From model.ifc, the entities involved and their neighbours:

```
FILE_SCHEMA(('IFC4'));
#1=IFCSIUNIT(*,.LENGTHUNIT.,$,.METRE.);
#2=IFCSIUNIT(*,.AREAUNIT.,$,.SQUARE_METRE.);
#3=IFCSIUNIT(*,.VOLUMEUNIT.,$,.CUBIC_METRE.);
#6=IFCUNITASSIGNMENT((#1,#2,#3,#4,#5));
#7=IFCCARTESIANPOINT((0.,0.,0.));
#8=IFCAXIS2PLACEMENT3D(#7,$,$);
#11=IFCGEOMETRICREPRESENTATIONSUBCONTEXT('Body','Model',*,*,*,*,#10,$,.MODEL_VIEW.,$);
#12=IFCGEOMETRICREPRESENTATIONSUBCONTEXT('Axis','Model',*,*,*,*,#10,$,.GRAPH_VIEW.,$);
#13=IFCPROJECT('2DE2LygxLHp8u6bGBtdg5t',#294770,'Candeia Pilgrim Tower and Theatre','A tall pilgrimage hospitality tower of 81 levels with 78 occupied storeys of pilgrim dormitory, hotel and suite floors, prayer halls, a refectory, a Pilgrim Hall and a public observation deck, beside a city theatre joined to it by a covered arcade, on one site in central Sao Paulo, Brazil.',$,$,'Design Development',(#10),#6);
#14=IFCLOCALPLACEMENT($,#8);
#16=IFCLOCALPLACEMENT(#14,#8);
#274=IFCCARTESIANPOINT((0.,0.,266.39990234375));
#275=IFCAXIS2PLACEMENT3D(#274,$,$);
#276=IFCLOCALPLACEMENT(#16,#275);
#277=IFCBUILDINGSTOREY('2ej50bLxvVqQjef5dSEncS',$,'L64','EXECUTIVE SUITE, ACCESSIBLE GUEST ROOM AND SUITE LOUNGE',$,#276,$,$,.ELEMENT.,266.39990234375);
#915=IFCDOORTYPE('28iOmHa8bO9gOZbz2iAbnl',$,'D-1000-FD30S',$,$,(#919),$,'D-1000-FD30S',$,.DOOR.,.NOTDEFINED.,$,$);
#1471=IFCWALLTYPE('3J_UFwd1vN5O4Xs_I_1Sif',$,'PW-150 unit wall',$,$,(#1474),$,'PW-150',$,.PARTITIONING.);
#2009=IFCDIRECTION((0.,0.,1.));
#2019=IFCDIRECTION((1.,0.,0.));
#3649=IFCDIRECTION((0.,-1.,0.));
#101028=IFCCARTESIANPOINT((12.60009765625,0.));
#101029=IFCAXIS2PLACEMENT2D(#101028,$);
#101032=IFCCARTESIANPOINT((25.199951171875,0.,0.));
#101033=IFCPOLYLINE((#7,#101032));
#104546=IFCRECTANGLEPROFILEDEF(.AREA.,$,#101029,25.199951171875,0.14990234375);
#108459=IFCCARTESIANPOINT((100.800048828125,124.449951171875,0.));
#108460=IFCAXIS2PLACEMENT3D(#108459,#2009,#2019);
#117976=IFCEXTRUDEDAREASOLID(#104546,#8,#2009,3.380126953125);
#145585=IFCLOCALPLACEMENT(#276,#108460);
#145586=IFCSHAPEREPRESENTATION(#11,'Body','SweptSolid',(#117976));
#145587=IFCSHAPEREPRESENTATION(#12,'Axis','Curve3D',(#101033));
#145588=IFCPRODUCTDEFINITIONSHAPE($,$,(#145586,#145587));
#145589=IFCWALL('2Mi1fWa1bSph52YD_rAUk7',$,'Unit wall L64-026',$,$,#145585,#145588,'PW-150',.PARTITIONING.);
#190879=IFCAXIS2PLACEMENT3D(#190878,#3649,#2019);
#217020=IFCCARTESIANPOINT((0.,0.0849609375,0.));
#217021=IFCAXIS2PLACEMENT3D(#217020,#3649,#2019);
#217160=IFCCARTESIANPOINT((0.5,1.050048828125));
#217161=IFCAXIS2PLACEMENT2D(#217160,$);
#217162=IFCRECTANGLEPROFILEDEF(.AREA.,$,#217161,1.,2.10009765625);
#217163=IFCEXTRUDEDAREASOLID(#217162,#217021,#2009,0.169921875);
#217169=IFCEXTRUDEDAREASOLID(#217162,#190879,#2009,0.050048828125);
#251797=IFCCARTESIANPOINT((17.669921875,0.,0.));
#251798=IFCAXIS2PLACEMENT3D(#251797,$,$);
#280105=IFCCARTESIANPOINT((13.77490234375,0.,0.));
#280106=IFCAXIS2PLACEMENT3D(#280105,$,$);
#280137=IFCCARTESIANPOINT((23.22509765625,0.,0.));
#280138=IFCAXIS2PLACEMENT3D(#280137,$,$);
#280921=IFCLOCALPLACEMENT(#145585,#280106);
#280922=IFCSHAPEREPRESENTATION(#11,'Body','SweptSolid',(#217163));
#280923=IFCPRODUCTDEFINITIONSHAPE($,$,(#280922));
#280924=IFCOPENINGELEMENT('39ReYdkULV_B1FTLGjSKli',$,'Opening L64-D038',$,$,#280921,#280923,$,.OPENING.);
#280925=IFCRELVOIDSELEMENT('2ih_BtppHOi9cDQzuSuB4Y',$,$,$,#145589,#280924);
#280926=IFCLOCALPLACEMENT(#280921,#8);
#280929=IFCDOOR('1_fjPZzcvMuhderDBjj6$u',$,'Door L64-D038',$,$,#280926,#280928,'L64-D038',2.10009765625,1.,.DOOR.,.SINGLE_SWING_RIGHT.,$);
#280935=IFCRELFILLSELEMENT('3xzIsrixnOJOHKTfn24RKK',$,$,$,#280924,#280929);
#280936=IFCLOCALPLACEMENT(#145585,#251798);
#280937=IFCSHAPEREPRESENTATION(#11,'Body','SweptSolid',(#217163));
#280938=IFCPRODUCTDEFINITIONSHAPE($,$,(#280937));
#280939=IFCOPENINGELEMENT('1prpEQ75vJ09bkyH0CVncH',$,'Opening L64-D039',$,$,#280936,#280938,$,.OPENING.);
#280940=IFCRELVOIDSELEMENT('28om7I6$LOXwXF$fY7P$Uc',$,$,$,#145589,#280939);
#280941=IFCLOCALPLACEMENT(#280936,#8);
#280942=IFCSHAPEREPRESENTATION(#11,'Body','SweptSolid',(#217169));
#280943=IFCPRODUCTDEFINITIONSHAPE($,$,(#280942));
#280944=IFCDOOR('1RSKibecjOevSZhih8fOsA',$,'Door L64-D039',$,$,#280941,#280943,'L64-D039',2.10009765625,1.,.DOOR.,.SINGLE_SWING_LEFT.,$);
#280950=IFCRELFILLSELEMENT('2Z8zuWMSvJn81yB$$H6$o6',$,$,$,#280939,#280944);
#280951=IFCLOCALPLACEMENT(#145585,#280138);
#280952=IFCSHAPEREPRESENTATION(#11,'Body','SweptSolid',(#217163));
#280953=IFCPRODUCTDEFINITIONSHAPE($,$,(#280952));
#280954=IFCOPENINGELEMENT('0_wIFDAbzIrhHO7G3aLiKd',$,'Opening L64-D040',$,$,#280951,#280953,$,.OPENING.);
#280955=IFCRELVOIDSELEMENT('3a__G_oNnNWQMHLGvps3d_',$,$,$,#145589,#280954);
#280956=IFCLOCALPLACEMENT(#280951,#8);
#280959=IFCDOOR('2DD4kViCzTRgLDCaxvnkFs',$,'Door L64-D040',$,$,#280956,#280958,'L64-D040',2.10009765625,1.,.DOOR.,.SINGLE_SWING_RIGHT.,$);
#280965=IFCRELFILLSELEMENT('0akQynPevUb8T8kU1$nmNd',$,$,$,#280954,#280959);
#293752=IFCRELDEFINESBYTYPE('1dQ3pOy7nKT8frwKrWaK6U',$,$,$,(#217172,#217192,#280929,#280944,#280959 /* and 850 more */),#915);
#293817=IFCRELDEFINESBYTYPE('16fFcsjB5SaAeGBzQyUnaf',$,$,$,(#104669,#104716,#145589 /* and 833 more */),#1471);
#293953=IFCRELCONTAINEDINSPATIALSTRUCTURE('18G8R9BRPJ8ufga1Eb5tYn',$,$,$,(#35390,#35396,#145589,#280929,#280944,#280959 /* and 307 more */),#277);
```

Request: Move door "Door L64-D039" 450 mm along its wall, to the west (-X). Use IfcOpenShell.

```python
import ifcopenshell
import ifcopenshell.api.geometry
import ifcopenshell.util.placement

model = ifcopenshell.open("model.ifc")

door = model.by_id(280944)
opening = door.FillsVoids[0].RelatingOpeningElement
wall = opening.VoidsElements[0].RelatingBuildingElement

wall_matrix = ifcopenshell.util.placement.get_local_placement(wall.ObjectPlacement)
shift = wall_matrix[:3, 0] * -0.45
before = ifcopenshell.util.placement.get_local_placement(door.ObjectPlacement)[:3, 3].copy()

# The door is placed relative to its opening, so it follows when the opening moves.
matrix = ifcopenshell.util.placement.get_local_placement(opening.ObjectPlacement)
matrix[:3, 3] += shift
ifcopenshell.api.geometry.edit_object_placement(
    model, product=opening, matrix=matrix, is_si=False, should_transform_children=True
)

after = ifcopenshell.util.placement.get_local_placement(door.ObjectPlacement)[:3, 3]
print("door moved by", (after - before).round(3) + 0.0)

model.write("model-out.ifc")
```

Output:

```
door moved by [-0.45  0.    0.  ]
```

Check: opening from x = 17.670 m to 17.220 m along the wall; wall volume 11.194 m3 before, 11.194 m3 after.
